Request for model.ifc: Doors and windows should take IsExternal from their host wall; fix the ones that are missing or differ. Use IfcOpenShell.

First a look at what the model holds.

```python
import ifcopenshell
import ifcopenshell.util.element

model = ifcopenshell.open("model.ifc")
print(model.schema)
seen = {}
for e in model.by_type("IfcDoor") + model.by_type("IfcWindow"):
    if not e.FillsVoids:
        continue
    host = e.FillsVoids[0].RelatingOpeningElement.VoidsElements[0].RelatingBuildingElement
    own = ifcopenshell.util.element.get_pset(e, f"Pset_{e.is_a()[3:].removesuffix('StandardCase')}Common", "IsExternal")
    wall = ifcopenshell.util.element.get_pset(host, "Pset_WallCommon", "IsExternal")
    seen[e.is_a(), own, wall] = seen.get((e.is_a(), own, wall), 0) + 1
for (cls, own, wall), count in sorted(seen.items(), key=str):
    print(count, cls, "IsExternal:", own, "| host wall:", wall)
```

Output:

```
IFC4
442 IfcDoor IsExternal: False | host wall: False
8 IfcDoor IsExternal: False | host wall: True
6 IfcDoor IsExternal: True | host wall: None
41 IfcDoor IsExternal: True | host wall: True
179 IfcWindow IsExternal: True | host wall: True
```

```python
import ifcopenshell
import ifcopenshell.api.pset
import ifcopenshell.util.element

model = ifcopenshell.open("model.ifc")

count = 0
for ifc_class, pset_name in (("IfcDoor", "Pset_DoorCommon"), ("IfcWindow", "Pset_WindowCommon")):
    for e in model.by_type(ifc_class):
        if not e.FillsVoids:
            continue
        host = e.FillsVoids[0].RelatingOpeningElement.VoidsElements[0].RelatingBuildingElement
        external = ifcopenshell.util.element.get_pset(host, "Pset_WallCommon", "IsExternal")
        if external is None or ifcopenshell.util.element.get_pset(e, pset_name, "IsExternal") == external:
            continue
        pset = ifcopenshell.api.pset.add_pset(model, product=e, name=pset_name)
        ifcopenshell.api.pset.edit_pset(model, pset=pset, properties={"IsExternal": external})
        count += 1

print(count, "updated")

model.write("model_updated.ifc")
```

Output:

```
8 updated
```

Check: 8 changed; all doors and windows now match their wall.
